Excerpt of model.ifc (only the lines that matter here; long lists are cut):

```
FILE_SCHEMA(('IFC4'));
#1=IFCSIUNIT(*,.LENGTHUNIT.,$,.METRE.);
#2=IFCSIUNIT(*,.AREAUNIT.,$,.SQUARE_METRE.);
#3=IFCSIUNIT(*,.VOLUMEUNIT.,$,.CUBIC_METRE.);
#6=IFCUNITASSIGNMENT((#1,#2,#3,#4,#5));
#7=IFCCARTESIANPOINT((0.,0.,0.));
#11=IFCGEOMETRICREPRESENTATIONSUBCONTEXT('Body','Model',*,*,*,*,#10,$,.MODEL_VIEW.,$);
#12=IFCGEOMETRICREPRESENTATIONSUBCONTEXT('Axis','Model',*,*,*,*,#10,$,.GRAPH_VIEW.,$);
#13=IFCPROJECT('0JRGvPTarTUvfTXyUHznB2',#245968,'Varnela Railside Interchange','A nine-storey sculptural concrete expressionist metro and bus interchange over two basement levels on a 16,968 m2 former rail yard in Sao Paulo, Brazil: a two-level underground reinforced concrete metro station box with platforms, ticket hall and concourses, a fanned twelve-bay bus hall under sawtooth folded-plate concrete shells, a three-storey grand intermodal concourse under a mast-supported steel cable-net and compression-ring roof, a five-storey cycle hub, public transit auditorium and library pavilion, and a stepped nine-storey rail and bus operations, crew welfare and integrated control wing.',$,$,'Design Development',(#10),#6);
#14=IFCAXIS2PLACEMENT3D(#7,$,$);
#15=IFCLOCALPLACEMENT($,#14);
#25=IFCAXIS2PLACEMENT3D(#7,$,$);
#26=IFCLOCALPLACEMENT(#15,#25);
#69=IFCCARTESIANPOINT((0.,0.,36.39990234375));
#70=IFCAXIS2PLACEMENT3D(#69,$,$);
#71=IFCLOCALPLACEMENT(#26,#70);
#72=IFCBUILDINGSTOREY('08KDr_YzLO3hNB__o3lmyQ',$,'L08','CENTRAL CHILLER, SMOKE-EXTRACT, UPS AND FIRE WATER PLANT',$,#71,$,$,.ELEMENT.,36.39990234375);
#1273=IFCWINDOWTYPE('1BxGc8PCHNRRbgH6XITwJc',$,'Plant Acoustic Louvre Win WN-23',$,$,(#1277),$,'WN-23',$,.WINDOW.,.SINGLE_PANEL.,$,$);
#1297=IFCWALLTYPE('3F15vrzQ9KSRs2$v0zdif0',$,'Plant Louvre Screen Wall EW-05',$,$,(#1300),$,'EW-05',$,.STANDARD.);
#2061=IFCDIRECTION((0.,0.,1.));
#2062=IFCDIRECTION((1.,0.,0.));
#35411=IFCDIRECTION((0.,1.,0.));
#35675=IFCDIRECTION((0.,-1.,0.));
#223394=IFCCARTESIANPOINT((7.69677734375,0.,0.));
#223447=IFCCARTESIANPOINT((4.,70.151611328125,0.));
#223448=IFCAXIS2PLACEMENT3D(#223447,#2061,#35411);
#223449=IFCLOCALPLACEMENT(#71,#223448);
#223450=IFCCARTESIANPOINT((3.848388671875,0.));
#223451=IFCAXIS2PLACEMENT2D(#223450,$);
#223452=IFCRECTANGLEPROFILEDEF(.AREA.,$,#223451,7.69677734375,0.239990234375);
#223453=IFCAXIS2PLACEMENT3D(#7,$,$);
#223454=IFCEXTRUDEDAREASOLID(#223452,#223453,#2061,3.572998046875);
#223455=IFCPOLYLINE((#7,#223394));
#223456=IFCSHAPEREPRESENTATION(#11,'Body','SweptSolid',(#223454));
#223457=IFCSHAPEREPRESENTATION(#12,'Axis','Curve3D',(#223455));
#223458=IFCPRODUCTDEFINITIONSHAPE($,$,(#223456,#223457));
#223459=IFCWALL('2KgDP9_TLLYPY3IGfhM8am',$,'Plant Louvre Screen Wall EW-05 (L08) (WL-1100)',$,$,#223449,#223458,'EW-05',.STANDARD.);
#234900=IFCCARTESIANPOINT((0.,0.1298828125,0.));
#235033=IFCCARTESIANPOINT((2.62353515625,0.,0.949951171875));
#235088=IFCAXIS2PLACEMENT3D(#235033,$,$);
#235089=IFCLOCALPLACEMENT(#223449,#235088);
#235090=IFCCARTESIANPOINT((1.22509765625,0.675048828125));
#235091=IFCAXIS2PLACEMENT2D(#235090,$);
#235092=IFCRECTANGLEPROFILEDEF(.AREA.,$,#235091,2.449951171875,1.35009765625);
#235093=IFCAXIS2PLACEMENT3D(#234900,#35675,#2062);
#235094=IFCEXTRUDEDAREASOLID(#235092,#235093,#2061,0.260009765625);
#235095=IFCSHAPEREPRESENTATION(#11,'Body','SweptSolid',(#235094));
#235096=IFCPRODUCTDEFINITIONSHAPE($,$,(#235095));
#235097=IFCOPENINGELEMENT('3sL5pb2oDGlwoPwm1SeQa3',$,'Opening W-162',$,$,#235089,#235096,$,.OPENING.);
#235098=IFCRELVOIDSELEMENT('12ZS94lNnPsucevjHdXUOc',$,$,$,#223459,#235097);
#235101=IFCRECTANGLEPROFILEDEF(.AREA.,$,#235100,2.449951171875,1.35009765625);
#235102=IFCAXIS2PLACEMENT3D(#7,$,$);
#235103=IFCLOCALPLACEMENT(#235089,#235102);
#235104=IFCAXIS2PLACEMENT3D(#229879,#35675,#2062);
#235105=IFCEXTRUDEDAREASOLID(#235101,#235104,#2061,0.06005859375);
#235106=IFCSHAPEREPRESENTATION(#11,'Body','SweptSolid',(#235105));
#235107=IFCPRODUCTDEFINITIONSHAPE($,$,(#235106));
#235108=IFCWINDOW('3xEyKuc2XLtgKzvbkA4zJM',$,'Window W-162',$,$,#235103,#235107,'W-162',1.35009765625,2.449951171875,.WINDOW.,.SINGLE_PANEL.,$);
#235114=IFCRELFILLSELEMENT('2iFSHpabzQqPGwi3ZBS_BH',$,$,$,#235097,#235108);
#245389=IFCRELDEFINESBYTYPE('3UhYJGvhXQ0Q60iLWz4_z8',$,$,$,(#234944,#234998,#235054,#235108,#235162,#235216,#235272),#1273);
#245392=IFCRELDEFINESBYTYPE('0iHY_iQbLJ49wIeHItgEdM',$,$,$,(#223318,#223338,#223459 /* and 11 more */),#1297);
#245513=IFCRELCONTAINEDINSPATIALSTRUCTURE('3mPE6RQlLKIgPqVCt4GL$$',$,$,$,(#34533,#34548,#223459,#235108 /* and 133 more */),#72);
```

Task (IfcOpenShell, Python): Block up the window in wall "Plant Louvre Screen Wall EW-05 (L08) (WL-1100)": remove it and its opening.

```python
import ifcopenshell
import ifcopenshell.api.feature
import ifcopenshell.api.root
import ifcopenshell.geom
import ifcopenshell.util.shape

model = ifcopenshell.open("model.ifc")
settings = ifcopenshell.geom.settings()


def volume(element):
    """Net volume in cubic metres, openings subtracted."""
    shape = ifcopenshell.geom.create_shape(settings, element)
    return ifcopenshell.util.shape.get_volume(shape.geometry)


window = model.by_guid("3xEyKuc2XLtgKzvbkA4zJM")
opening = window.FillsVoids[0].RelatingOpeningElement
wall = opening.VoidsElements[0].RelatingBuildingElement
before = volume(wall)

ifcopenshell.api.root.remove_product(model, product=window)
ifcopenshell.api.feature.remove_feature(model, feature=opening)

after = volume(wall)

print(f"wall volume {before:.3f} -> {after:.3f} m3")

model.write("model_updated.ifc")
```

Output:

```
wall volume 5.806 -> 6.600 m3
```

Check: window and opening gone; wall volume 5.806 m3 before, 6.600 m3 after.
